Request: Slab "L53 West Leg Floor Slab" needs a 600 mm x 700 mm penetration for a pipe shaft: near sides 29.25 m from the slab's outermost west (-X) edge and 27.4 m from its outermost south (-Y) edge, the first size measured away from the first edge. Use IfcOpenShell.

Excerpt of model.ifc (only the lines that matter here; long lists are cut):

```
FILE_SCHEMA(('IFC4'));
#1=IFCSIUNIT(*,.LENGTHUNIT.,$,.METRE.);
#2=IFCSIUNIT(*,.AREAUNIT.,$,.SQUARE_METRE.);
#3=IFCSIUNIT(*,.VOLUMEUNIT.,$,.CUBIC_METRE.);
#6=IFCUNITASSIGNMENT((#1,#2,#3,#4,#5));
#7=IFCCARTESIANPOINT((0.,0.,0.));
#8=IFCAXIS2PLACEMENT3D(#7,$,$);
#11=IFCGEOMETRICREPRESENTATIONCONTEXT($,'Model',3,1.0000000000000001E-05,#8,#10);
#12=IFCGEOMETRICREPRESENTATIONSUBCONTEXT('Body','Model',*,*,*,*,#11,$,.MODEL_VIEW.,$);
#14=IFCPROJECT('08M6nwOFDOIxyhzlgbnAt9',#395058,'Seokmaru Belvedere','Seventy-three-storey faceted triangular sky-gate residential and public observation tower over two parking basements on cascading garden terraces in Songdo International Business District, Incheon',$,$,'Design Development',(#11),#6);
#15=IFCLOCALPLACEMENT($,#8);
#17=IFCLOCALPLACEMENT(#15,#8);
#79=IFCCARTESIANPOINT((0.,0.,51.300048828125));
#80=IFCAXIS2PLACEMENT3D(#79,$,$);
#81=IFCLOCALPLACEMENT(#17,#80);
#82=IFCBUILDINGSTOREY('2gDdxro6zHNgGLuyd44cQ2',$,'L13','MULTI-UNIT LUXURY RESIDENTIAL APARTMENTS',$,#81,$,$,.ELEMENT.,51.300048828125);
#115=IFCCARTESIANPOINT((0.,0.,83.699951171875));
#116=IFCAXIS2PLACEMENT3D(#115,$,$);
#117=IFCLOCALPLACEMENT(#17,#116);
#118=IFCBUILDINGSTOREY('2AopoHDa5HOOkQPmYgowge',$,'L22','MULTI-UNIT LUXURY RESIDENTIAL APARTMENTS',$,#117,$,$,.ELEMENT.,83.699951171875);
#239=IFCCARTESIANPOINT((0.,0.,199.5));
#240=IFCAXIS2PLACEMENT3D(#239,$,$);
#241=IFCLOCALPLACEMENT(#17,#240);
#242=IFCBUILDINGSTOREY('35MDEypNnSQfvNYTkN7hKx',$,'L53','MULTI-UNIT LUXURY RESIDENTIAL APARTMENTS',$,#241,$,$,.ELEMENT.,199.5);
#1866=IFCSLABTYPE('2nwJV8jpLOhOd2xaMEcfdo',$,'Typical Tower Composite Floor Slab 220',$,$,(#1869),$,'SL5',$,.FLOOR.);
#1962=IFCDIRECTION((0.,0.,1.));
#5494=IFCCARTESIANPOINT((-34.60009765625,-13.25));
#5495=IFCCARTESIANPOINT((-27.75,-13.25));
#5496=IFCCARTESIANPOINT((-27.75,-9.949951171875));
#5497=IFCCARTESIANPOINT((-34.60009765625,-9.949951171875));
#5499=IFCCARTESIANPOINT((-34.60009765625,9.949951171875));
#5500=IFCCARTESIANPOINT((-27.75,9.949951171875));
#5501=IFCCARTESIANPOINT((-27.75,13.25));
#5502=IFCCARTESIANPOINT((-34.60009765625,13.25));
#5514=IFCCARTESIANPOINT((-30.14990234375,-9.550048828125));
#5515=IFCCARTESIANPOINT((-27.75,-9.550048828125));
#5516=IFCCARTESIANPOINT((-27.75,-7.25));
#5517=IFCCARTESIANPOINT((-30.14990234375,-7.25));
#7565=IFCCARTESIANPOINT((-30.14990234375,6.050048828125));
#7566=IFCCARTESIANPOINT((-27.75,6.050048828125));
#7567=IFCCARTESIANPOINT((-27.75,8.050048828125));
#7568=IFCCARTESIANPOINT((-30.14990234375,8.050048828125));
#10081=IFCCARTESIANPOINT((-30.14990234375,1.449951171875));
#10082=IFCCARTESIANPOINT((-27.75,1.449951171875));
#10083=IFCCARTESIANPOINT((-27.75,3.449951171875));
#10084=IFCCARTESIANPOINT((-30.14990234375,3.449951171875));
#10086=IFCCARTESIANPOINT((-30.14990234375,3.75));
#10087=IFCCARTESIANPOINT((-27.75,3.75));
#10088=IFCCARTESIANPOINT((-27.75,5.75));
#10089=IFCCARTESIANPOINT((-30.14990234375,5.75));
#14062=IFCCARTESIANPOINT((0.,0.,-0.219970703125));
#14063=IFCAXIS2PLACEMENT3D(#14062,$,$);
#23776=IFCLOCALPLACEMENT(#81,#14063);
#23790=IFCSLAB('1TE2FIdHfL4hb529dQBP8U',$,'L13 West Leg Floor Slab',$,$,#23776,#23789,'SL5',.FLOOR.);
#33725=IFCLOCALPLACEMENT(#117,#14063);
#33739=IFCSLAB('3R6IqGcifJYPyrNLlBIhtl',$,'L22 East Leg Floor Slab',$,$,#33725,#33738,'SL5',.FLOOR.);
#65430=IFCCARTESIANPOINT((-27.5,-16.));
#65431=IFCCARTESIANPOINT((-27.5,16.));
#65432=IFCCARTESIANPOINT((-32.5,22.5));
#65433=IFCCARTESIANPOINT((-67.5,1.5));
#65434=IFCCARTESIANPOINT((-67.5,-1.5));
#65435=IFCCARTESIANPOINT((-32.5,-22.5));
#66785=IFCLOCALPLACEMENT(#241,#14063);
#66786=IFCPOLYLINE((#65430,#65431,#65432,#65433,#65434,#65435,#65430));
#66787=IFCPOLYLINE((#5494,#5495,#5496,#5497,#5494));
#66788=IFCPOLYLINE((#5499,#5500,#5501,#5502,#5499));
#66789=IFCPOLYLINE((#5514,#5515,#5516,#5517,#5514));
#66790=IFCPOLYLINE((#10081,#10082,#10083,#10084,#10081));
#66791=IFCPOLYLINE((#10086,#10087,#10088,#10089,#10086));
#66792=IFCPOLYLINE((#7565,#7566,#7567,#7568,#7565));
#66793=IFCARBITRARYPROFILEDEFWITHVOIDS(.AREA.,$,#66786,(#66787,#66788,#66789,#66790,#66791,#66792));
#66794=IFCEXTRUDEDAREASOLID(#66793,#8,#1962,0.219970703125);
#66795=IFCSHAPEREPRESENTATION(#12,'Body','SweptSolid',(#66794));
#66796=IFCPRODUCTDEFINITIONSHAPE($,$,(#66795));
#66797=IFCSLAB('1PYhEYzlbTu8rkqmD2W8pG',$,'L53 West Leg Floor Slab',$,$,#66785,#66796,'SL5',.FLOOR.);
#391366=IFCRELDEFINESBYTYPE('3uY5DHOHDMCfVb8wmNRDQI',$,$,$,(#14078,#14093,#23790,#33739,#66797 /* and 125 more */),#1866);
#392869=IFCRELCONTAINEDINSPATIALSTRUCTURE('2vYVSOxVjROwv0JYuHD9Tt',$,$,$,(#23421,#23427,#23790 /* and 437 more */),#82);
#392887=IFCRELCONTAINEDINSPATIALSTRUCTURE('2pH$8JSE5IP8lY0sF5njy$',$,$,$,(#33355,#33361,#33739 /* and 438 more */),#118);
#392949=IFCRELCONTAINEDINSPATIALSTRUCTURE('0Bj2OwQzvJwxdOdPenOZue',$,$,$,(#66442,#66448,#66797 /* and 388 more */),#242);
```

```python
import numpy as np
import ifcopenshell
import ifcopenshell.api.feature
import ifcopenshell.api.geometry
import ifcopenshell.api.root
import ifcopenshell.geom
import ifcopenshell.util.placement
import ifcopenshell.util.representation
import ifcopenshell.util.shape
import ifcopenshell.util.unit

model = ifcopenshell.open("model.ifc")
unit_scale = ifcopenshell.util.unit.calculate_unit_scale(model)
settings = ifcopenshell.geom.settings()


def volume(element):
    """Net volume in cubic metres, openings subtracted."""
    shape = ifcopenshell.geom.create_shape(settings, element)
    return ifcopenshell.util.shape.get_volume(shape.geometry)


slab = model.by_guid("1PYhEYzlbTu8rkqmD2W8pG")
before = volume(slab)

# Extent in the slab's own axes, in metres. The edges named are its -X and -Y sides.
slab_shape = ifcopenshell.geom.create_shape(settings, slab)
vertices = ifcopenshell.util.shape.get_vertices(slab_shape.geometry)
x_min, y_min, bottom = vertices.min(axis=0)
top = vertices[:, 2].max()

opening = ifcopenshell.api.root.create_entity(model, ifc_class="IfcOpeningElement", name="Pipe shaft opening", predefined_type="OPENING")
context = ifcopenshell.util.representation.get_context(model, "Model", "Body", "MODEL_VIEW")
width, depth = 0.6, 0.7
outline = [(0.0, 0.0), (width, 0.0), (width, depth), (0.0, depth), (0.0, 0.0)]
# Overshoot both faces by 50 mm so the cut is clean.
shape = ifcopenshell.api.geometry.add_slab_representation(
    model, context=context, depth=top - bottom + 0.1, polyline=outline
)
ifcopenshell.api.geometry.assign_representation(model, product=opening, representation=shape)

matrix = ifcopenshell.util.placement.get_local_placement(slab.ObjectPlacement)
matrix[:, 3] = matrix @ np.append(np.array([x_min + 29.25, y_min + 27.4, bottom - 0.05]) / unit_scale, 1.0)
ifcopenshell.api.geometry.edit_object_placement(model, product=opening, matrix=matrix, is_si=False)
ifcopenshell.api.feature.add_feature(model, feature=opening, element=slab)

after = volume(slab)

print(f"slab volume {before:.3f} -> {after:.3f} m3")

model.write("model_edited.ifc")
```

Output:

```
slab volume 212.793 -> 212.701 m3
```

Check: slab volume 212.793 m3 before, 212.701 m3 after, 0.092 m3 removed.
